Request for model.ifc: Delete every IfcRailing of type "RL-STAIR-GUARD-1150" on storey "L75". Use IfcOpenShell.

First a look at what the model holds.

```python
import ifcopenshell
import ifcopenshell.util.element

model = ifcopenshell.open("model.ifc")
print(model.schema)
storey = next(s for s in model.by_type("IfcBuildingStorey") if s.Name == "L75")
railings = [e for e in ifcopenshell.util.element.get_decomposition(storey) if e.is_a("IfcRailing")]
seen = {}
for e in railings:
    element_type = ifcopenshell.util.element.get_type(e)
    name = element_type.Name if element_type not in (None, e) else None
    seen[name] = seen.get(name, 0) + 1
for name, count in sorted(seen.items(), key=str):
    print(count, "x", name)
```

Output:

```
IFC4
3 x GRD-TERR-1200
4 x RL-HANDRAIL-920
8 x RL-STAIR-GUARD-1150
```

```python
import ifcopenshell
import ifcopenshell.api.root
import ifcopenshell.util.element

model = ifcopenshell.open("model.ifc")

storey = next(s for s in model.by_type("IfcBuildingStorey") if s.Name == "L75")
railings = [e for e in ifcopenshell.util.element.get_decomposition(storey) if e.is_a("IfcRailing")]
targets = [e for e in railings if (t := ifcopenshell.util.element.get_type(e)) not in (None, e) and t.Name == "RL-STAIR-GUARD-1150"]

for e in targets:
    ifcopenshell.api.root.remove_product(model, product=e)
print(len(targets), "removed")

model.write("model-out.ifc")
```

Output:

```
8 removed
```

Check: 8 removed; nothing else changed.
